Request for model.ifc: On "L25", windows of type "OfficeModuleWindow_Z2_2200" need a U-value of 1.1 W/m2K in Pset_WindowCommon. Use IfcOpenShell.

First a look at what the model holds.

```python
import ifcopenshell
import ifcopenshell.util.element

model = ifcopenshell.open("model.ifc")
print(model.schema)
storey = next(s for s in model.by_type("IfcBuildingStorey") if s.Name == "L25")
windows = [e for e in ifcopenshell.util.element.get_decomposition(storey) if e.is_a("IfcWindow")]
seen = {}
for e in windows:
    element_type = ifcopenshell.util.element.get_type(e)
    key = (element_type.Name if element_type != e and element_type else None, ifcopenshell.util.element.get_pset(e, "Pset_WindowCommon", "ThermalTransmittance"))
    seen[key] = seen.get(key, 0) + 1
for (name, value), count in sorted(seen.items(), key=str):
    print(count, "x", name, "|", value)
```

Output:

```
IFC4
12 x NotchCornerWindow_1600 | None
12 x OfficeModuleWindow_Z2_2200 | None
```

```python
import ifcopenshell
import ifcopenshell.api.pset
import ifcopenshell.util.element

model = ifcopenshell.open("model.ifc")

storey = next(s for s in model.by_type("IfcBuildingStorey") if s.Name == "L25")
windows = [e for e in ifcopenshell.util.element.get_decomposition(storey) if e.is_a("IfcWindow")]

count = 0
for e in windows:
    element_type = ifcopenshell.util.element.get_type(e)
    if element_type in (None, e) or element_type.Name != "OfficeModuleWindow_Z2_2200":
        continue
    # add_pset returns the element's existing set when there is one.
    pset = ifcopenshell.api.pset.add_pset(model, product=e, name="Pset_WindowCommon")
    ifcopenshell.api.pset.edit_pset(model, pset=pset, properties={"ThermalTransmittance": 1.1})
    count += 1

print(count, "windows updated")

model.write("model_updated.ifc")
```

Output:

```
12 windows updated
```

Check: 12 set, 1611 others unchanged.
